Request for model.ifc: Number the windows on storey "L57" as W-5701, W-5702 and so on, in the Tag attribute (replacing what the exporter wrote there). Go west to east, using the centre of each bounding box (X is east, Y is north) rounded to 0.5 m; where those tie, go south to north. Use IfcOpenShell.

First a look at what the model holds.

```python
import ifcopenshell
import ifcopenshell.util.element
import ifcopenshell.util.placement

model = ifcopenshell.open("model.ifc")
print(model.schema)
storey = next(s for s in model.by_type("IfcBuildingStorey") if s.Name == "L57")
windows = [e for e in ifcopenshell.util.element.get_decomposition(storey) if e.is_a("IfcWindow")]
for e in sorted(windows, key=lambda e: e.id()):
    origin = ifcopenshell.util.placement.get_local_placement(e.ObjectPlacement)[:3, 3]
    print(e.id(), e.Tag, e.Name, origin.round(2) + 0.0, sep=" | ")
```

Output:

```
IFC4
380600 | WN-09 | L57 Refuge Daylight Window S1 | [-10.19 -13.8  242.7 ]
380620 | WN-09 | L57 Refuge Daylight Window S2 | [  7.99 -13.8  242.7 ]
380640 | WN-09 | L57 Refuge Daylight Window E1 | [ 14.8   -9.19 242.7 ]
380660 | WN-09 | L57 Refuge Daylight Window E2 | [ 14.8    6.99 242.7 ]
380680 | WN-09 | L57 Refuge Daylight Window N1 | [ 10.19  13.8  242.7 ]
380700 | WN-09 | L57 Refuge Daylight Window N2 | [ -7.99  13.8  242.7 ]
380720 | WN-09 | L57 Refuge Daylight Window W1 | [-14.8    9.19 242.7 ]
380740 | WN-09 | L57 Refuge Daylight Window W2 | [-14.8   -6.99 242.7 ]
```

```python
import ifcopenshell
import ifcopenshell.geom
import ifcopenshell.util.element
import ifcopenshell.util.shape

model = ifcopenshell.open("model.ifc")
settings = ifcopenshell.geom.settings()
settings.set("use-world-coords", True)


def centre(element):
    shape = ifcopenshell.geom.create_shape(settings, element)
    return ifcopenshell.util.shape.get_bbox_centroid(shape.geometry)


storey = next(s for s in model.by_type("IfcBuildingStorey") if s.Name == "L57")
windows = [e for e in ifcopenshell.util.element.get_decomposition(storey) if e.is_a("IfcWindow")]

# Insertion points can sit at a corner or the storey origin, so sort by the geometry (in metres).
centres = {e: centre(e) for e in windows}
windows.sort(key=lambda e: (round(centres[e][0] / 0.5), centres[e][1]))

for i, e in enumerate(windows, start=1):
    number = f"W-57{i:02d}"
    e.Tag = number
    print(e.id(), number)

model.write("model_updated.ifc")
```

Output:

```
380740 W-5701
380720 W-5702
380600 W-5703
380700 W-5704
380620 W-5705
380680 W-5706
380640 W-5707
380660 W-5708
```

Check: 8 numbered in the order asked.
